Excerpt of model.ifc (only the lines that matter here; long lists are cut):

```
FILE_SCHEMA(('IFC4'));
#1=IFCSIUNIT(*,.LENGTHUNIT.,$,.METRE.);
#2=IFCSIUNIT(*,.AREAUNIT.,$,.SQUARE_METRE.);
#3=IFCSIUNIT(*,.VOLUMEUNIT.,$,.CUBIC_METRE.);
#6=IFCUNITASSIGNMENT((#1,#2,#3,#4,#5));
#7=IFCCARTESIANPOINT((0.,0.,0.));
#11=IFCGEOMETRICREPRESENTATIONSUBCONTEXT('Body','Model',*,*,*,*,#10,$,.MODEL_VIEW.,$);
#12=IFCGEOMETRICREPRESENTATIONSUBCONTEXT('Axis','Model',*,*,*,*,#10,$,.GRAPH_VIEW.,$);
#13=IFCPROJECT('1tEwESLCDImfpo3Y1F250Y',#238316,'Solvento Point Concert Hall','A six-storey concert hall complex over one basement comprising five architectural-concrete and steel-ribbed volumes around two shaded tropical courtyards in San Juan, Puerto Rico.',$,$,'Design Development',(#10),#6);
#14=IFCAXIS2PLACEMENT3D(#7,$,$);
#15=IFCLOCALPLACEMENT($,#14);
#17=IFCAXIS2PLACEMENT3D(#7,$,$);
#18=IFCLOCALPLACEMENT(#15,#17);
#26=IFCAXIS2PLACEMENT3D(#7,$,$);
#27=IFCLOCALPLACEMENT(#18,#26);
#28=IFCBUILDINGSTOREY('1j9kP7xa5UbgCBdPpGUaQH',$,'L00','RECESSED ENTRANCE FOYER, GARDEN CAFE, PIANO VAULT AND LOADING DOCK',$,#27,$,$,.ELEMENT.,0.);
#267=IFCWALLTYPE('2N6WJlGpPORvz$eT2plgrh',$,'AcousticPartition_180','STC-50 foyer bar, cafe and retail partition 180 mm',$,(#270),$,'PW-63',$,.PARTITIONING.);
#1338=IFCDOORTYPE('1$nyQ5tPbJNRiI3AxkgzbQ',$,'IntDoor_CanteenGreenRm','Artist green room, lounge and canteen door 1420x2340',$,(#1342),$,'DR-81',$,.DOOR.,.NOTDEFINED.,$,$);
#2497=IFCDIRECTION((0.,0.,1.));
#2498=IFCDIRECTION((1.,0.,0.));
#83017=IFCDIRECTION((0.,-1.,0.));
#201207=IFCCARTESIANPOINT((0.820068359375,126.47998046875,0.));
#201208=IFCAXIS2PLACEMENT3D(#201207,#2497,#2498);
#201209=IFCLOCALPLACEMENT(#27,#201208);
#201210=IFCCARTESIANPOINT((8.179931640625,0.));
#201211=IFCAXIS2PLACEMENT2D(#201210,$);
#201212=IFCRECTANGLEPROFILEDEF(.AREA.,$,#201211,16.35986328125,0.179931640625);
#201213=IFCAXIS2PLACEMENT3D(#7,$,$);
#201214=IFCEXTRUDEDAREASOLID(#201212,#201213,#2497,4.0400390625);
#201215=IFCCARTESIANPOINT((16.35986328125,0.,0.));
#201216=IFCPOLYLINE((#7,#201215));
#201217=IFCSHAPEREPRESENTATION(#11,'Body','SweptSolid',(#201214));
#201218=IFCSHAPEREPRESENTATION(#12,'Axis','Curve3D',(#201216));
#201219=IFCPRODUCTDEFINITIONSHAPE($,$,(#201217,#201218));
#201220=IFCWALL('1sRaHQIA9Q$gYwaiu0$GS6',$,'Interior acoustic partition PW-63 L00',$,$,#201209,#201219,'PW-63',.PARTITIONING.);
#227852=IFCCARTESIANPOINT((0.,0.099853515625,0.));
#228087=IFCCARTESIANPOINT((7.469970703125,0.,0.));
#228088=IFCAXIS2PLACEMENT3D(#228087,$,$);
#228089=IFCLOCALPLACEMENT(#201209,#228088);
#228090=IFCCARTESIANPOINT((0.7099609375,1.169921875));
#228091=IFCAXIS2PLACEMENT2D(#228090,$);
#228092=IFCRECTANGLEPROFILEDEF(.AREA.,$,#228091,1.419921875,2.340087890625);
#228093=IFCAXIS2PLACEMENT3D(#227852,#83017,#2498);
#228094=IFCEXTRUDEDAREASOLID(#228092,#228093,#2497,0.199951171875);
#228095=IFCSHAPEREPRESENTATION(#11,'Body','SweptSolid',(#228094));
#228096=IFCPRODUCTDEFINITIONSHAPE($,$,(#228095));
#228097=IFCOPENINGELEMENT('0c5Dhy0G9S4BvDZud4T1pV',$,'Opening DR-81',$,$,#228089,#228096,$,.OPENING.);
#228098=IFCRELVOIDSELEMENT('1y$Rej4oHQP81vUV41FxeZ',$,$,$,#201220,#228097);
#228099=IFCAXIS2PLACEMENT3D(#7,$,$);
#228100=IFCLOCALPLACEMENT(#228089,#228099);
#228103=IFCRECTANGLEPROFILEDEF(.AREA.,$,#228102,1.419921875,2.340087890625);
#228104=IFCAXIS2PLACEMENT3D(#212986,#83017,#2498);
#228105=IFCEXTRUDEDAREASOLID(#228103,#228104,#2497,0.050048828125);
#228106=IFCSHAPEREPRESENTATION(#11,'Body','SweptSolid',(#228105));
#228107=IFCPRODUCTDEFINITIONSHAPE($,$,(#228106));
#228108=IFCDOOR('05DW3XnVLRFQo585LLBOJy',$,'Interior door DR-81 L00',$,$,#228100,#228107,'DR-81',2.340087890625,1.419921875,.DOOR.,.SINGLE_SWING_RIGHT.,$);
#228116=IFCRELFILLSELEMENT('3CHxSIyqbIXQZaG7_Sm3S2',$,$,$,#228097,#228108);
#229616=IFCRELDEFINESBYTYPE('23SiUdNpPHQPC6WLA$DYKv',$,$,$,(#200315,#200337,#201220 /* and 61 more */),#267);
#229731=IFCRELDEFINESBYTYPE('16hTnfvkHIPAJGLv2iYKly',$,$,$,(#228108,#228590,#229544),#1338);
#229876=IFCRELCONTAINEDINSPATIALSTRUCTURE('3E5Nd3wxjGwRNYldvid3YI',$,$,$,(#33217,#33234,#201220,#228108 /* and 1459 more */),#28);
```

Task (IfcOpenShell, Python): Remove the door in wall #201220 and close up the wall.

```python
import ifcopenshell
import ifcopenshell.api.feature
import ifcopenshell.api.root
import ifcopenshell.geom
import ifcopenshell.util.shape

model = ifcopenshell.open("model.ifc")
settings = ifcopenshell.geom.settings()


def volume(element):
    """Net volume in cubic metres, openings subtracted."""
    shape = ifcopenshell.geom.create_shape(settings, element)
    return ifcopenshell.util.shape.get_volume(shape.geometry)


door = model.by_id(228108)
opening = door.FillsVoids[0].RelatingOpeningElement
wall = opening.VoidsElements[0].RelatingBuildingElement
before = volume(wall)

ifcopenshell.api.root.remove_product(model, product=door)
ifcopenshell.api.feature.remove_feature(model, feature=opening)

after = volume(wall)

print(f"wall volume {before:.3f} -> {after:.3f} m3")

model.write("model_updated.ifc")
```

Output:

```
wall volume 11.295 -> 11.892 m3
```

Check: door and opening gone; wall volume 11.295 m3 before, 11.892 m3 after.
